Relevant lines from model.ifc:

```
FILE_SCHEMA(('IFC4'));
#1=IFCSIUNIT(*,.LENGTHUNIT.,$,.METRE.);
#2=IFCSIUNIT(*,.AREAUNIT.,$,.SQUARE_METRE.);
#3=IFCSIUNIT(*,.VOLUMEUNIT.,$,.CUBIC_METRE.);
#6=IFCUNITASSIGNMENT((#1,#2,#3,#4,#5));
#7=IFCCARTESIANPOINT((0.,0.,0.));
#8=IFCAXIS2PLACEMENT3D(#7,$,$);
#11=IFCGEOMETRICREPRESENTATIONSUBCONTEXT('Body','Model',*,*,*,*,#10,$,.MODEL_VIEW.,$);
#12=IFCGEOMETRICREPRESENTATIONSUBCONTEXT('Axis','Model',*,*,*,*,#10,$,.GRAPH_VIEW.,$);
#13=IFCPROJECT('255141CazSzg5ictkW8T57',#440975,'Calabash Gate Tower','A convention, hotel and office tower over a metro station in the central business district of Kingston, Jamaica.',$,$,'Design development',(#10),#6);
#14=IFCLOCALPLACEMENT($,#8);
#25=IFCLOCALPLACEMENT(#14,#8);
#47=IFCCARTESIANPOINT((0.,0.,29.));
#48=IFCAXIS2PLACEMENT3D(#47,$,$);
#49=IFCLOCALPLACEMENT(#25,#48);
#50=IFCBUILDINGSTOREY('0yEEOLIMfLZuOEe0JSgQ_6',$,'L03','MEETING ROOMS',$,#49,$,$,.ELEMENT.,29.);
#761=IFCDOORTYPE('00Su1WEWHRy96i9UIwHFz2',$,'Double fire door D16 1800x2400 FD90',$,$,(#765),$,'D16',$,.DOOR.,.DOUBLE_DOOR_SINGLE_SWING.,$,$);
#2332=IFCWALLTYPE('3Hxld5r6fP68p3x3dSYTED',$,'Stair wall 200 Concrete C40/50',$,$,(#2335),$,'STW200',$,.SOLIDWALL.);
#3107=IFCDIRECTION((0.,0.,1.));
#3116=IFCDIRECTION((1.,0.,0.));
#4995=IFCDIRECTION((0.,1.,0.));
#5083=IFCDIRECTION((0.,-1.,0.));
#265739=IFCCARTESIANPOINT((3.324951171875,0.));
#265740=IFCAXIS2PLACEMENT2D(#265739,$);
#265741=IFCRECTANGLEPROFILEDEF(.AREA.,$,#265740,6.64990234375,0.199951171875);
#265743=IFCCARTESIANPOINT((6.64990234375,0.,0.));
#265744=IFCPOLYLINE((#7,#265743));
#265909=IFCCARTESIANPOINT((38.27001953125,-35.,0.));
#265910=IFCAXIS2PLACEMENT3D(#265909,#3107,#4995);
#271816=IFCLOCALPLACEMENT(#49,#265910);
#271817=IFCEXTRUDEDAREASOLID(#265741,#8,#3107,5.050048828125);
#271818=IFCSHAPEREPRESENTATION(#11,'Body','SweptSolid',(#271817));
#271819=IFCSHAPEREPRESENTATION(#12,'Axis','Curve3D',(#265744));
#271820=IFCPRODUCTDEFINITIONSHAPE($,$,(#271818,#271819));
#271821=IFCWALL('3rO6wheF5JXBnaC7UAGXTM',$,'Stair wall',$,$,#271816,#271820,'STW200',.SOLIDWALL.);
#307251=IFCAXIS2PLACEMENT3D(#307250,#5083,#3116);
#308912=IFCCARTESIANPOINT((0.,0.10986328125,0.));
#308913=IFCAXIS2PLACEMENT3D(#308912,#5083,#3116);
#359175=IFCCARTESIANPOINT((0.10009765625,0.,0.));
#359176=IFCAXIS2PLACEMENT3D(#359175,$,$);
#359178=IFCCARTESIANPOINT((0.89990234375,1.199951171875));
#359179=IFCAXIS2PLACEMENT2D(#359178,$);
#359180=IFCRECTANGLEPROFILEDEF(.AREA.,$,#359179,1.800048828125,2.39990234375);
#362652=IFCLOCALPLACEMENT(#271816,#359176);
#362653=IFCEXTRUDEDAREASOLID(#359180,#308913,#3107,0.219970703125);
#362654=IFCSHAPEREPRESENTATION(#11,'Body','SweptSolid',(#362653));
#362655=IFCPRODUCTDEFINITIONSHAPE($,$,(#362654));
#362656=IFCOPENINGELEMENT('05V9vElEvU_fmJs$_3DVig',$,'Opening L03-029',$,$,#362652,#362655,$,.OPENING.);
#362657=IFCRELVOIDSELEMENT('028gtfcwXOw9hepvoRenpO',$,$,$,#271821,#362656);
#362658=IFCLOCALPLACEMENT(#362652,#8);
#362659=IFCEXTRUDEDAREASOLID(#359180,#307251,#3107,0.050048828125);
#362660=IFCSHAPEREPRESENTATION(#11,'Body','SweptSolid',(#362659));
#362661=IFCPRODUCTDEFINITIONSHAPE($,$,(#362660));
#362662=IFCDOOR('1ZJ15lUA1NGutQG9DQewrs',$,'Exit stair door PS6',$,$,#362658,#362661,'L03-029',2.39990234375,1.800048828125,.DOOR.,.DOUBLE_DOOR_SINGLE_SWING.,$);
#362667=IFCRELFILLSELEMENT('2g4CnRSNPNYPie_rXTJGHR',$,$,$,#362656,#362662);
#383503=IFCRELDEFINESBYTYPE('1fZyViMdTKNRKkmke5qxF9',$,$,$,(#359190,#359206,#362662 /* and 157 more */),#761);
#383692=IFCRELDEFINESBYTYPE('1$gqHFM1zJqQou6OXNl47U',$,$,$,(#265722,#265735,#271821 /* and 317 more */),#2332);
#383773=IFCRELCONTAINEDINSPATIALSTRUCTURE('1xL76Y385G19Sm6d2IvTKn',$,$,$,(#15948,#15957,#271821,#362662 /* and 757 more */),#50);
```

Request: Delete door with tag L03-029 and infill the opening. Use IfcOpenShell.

```python
import ifcopenshell
import ifcopenshell.api.feature
import ifcopenshell.api.root
import ifcopenshell.geom
import ifcopenshell.util.shape

model = ifcopenshell.open("model.ifc")
settings = ifcopenshell.geom.settings()


def volume(element):
    """Net volume in cubic metres, openings subtracted."""
    shape = ifcopenshell.geom.create_shape(settings, element)
    return ifcopenshell.util.shape.get_volume(shape.geometry)


door = model.by_guid("1ZJ15lUA1NGutQG9DQewrs")
opening = door.FillsVoids[0].RelatingOpeningElement
wall = opening.VoidsElements[0].RelatingBuildingElement
before = volume(wall)

ifcopenshell.api.root.remove_product(model, product=door)
ifcopenshell.api.feature.remove_feature(model, feature=opening)

after = volume(wall)

print(f"wall volume {before:.3f} -> {after:.3f} m3")

model.write("model_v2.ifc")
```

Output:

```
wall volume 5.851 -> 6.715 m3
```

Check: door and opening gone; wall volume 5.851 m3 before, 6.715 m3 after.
